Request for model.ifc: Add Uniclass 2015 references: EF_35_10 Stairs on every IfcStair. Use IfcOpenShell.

First a look at what the model holds.

```python
import ifcopenshell

model = ifcopenshell.open("model.ifc")
print(model.schema)
print("classifications:", [c.Name for c in model.by_type("IfcClassification")])
for ifc_class in ("IfcDoor", "IfcRoof", "IfcStair", "IfcWall", "IfcWindow"):
    print(ifc_class, len(model.by_type(ifc_class)))
```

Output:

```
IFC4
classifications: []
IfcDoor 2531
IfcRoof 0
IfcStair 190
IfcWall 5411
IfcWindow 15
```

```python
import ifcopenshell
import ifcopenshell.api.classification

model = ifcopenshell.open("model.ifc")

system = ifcopenshell.api.classification.add_classification(model, classification="Uniclass 2015")

codes = {
    "IfcStair": ("EF_35_10", "Stairs"),
}
for ifc_class, (code, name) in codes.items():
    products = model.by_type(ifc_class)
    ifcopenshell.api.classification.add_reference(
        model, products=products, classification=system, identification=code, name=name
    )
    print(code, len(products))

model.write("model-out.ifc")
```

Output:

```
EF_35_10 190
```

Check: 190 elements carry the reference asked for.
